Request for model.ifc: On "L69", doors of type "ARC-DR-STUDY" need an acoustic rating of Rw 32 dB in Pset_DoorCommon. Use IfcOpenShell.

First a look at what the model holds.

```python
import ifcopenshell
import ifcopenshell.util.element

model = ifcopenshell.open("model.ifc")
print(model.schema)
storey = next(s for s in model.by_type("IfcBuildingStorey") if s.Name == "L69")
doors = [e for e in ifcopenshell.util.element.get_decomposition(storey) if e.is_a("IfcDoor")]
seen = {}
for e in doors:
    element_type = ifcopenshell.util.element.get_type(e)
    key = (element_type.Name if element_type != e and element_type else None, ifcopenshell.util.element.get_pset(e, "Pset_DoorCommon", "AcousticRating"))
    seen[key] = seen.get(key, 0) + 1
for (name, value), count in sorted(seen.items(), key=str):
    print(count, "x", name, "|", value)
```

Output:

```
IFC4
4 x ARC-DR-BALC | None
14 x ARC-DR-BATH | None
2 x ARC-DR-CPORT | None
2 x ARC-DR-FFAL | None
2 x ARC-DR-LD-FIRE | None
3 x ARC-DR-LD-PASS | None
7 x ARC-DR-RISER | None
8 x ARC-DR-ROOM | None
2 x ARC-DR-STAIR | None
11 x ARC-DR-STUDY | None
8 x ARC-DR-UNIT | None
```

```python
import ifcopenshell
import ifcopenshell.api.pset
import ifcopenshell.util.element

model = ifcopenshell.open("model.ifc")

storey = next(s for s in model.by_type("IfcBuildingStorey") if s.Name == "L69")
doors = [e for e in ifcopenshell.util.element.get_decomposition(storey) if e.is_a("IfcDoor")]

count = 0
for e in doors:
    element_type = ifcopenshell.util.element.get_type(e)
    if element_type in (None, e) or element_type.Name != "ARC-DR-STUDY":
        continue
    # add_pset returns the element's existing set when there is one.
    pset = ifcopenshell.api.pset.add_pset(model, product=e, name="Pset_DoorCommon")
    ifcopenshell.api.pset.edit_pset(model, pset=pset, properties={"AcousticRating": "Rw 32 dB"})
    count += 1

print(count, "doors updated")

model.write("model_edited.ifc")
```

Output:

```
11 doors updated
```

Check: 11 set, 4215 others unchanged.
